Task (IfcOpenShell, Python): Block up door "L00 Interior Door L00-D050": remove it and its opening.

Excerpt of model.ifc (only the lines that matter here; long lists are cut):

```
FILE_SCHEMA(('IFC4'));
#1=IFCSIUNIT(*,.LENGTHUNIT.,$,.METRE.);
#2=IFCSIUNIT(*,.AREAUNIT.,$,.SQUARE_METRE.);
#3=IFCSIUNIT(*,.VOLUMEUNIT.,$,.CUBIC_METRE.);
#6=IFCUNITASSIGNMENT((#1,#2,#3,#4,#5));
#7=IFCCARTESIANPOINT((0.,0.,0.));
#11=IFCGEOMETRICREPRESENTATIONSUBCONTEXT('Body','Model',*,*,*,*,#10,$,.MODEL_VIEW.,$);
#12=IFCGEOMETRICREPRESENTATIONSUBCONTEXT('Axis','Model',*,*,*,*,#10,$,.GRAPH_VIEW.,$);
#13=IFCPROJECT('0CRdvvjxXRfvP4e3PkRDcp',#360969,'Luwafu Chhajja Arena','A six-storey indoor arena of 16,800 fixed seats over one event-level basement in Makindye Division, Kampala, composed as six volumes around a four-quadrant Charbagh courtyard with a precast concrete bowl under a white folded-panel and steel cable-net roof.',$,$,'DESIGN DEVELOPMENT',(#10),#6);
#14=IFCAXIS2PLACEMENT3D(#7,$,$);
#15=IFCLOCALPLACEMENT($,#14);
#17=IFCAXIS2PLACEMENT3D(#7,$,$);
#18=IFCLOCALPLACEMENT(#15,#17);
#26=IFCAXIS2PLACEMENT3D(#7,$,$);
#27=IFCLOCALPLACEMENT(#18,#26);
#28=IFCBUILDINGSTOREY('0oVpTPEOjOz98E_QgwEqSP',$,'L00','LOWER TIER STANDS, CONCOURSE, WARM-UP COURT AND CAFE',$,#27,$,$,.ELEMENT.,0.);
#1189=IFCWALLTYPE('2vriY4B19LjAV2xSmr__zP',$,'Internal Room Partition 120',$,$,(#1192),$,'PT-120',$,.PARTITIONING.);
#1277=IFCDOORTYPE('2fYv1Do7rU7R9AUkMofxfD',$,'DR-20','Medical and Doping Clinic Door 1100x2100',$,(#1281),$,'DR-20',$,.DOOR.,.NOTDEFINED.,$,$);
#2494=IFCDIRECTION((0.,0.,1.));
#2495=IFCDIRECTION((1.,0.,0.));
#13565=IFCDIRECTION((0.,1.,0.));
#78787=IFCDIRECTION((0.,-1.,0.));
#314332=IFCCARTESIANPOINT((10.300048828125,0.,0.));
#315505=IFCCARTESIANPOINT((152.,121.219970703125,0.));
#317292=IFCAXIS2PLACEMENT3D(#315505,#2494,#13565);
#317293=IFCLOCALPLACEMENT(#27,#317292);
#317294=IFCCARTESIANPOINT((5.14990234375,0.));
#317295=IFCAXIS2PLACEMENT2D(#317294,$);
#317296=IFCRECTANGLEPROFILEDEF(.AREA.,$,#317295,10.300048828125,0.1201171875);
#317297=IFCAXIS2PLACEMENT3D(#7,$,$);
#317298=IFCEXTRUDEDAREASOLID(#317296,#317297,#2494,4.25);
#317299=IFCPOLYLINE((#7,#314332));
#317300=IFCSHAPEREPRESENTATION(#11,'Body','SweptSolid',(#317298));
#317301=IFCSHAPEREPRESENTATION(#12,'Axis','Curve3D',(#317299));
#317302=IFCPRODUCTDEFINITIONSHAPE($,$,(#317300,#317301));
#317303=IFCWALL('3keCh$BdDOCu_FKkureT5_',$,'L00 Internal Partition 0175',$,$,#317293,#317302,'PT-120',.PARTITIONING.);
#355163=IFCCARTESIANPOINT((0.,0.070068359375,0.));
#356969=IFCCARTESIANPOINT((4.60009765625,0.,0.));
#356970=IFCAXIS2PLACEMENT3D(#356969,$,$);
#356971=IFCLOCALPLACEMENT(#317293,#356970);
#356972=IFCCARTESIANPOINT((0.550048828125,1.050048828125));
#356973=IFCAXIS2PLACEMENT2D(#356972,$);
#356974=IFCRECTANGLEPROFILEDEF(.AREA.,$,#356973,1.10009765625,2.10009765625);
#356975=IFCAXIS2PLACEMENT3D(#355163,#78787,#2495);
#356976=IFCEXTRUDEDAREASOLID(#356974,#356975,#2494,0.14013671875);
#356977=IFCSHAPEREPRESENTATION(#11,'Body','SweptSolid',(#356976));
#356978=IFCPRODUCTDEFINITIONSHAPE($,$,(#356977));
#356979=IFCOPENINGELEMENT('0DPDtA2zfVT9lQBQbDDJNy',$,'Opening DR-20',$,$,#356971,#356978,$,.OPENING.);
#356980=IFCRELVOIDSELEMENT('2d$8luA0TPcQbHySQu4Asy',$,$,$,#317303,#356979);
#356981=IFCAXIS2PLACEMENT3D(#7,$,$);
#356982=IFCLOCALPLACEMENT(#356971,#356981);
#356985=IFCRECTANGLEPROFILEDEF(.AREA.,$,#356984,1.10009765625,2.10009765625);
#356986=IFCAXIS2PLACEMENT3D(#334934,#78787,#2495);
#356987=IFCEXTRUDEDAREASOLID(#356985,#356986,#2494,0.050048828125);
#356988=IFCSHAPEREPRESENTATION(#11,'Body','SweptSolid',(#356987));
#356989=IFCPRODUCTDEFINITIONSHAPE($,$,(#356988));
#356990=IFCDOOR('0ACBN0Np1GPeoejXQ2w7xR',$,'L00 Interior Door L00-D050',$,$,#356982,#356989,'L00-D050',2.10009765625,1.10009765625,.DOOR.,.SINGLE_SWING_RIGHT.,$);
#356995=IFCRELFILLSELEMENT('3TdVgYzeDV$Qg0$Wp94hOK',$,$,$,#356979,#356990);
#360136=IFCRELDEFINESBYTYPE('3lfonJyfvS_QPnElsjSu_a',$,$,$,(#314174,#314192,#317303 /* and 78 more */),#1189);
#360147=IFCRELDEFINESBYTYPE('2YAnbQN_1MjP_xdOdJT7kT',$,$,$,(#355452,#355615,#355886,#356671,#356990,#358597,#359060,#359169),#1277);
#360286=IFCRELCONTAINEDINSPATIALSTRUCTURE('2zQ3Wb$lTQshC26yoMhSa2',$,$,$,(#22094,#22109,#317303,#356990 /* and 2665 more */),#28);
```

```python
import ifcopenshell
import ifcopenshell.api.feature
import ifcopenshell.api.root
import ifcopenshell.geom
import ifcopenshell.util.shape

model = ifcopenshell.open("model.ifc")
settings = ifcopenshell.geom.settings()


def volume(element):
    """Net volume in cubic metres, openings subtracted."""
    shape = ifcopenshell.geom.create_shape(settings, element)
    return ifcopenshell.util.shape.get_volume(shape.geometry)


door = model.by_guid("0ACBN0Np1GPeoejXQ2w7xR")
opening = door.FillsVoids[0].RelatingOpeningElement
wall = opening.VoidsElements[0].RelatingBuildingElement
before = volume(wall)

ifcopenshell.api.root.remove_product(model, product=door)
ifcopenshell.api.feature.remove_feature(model, feature=opening)

after = volume(wall)

print(f"wall volume {before:.3f} -> {after:.3f} m3")

model.write("model_edited.ifc")
```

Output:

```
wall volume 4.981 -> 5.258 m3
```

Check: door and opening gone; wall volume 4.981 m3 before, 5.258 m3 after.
